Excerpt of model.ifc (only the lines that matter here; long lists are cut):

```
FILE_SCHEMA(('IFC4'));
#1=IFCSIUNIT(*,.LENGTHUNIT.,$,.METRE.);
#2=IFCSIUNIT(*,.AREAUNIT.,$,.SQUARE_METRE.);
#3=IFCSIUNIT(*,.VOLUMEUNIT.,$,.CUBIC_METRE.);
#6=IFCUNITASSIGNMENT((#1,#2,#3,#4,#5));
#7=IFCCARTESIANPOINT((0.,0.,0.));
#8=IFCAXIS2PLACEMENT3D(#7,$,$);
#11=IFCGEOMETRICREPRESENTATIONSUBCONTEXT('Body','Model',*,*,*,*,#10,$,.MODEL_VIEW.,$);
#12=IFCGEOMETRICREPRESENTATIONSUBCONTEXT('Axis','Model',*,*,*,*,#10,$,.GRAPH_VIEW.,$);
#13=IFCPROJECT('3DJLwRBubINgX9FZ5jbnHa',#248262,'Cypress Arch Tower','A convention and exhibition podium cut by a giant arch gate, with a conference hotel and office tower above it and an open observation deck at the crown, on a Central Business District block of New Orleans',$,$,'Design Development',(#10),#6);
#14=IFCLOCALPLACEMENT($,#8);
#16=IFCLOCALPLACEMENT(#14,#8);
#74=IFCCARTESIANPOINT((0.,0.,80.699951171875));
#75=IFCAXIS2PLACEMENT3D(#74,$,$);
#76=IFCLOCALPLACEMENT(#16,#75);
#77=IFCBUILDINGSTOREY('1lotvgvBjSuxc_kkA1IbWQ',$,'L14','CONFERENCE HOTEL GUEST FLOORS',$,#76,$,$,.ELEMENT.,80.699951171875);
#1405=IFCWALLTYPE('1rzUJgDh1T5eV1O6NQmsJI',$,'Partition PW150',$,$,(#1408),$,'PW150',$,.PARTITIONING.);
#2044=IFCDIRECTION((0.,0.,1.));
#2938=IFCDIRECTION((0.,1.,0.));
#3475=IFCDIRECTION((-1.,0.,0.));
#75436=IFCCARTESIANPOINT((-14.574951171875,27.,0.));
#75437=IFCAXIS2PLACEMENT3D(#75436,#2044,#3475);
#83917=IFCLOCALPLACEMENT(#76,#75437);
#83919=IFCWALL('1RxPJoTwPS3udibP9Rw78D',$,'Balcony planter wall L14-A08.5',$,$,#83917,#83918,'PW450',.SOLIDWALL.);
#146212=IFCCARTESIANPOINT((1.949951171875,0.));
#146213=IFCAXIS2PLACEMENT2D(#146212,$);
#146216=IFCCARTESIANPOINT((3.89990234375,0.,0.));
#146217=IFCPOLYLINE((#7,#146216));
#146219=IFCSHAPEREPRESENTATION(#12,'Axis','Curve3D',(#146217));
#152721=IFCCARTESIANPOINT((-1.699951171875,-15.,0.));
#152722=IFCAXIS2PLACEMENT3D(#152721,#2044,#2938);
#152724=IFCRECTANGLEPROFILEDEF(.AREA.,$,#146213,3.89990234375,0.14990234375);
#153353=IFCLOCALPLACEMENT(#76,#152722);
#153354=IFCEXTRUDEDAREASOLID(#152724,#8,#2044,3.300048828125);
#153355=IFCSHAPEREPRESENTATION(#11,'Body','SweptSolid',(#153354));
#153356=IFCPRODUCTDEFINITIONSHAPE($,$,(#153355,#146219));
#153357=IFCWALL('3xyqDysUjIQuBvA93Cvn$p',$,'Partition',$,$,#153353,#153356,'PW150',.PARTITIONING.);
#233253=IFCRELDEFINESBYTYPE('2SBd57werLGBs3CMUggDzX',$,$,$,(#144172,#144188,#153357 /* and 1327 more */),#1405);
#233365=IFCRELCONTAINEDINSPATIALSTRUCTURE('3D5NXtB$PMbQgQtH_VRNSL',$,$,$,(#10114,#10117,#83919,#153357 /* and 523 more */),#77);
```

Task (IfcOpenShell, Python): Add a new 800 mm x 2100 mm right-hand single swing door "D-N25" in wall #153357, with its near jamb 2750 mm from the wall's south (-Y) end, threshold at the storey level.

```python
import numpy as np
import ifcopenshell
import ifcopenshell.api.feature
import ifcopenshell.api.geometry
import ifcopenshell.api.root
import ifcopenshell.api.spatial
import ifcopenshell.geom
import ifcopenshell.util.element
import ifcopenshell.util.placement
import ifcopenshell.util.representation
import ifcopenshell.util.shape
import ifcopenshell.util.unit

model = ifcopenshell.open("model.ifc")
unit_scale = ifcopenshell.util.unit.calculate_unit_scale(model)
settings = ifcopenshell.geom.settings()


def volume(element):
    """Net volume in cubic metres, openings subtracted."""
    shape = ifcopenshell.geom.create_shape(settings, element)
    return ifcopenshell.util.shape.get_volume(shape.geometry)


wall = model.by_guid("3xyqDysUjIQuBvA93Cvn$p")
storey = ifcopenshell.util.element.get_container(wall, ifc_class="IfcBuildingStorey")
context = ifcopenshell.util.representation.get_context(model, "Model", "Body", "MODEL_VIEW")
before = volume(wall)

width, height, from_end, sill = 0.8, 2.1, 2.75, 0.0  # metres

# The wall runs along its own X axis, and the end named is its -X end.
wall_shape = ifcopenshell.geom.create_shape(settings, wall)
x, y, z = ifcopenshell.util.shape.get_vertices(wall_shape.geometry).T
start = x.min() + from_end
face, thickness = float(y.min()), float(y.max() - y.min())
wall_matrix = ifcopenshell.util.placement.get_local_placement(wall.ObjectPlacement)
level = ifcopenshell.util.placement.get_local_placement(storey.ObjectPlacement)[2, 3]


def in_wall(x, y):
    """Placement at x, y metres in the wall's axes, at sill height."""
    matrix = wall_matrix.copy()
    matrix[:, 3] = wall_matrix @ np.array([x / unit_scale, y / unit_scale, 0.0, 1.0])
    matrix[2, 3] = level + sill / unit_scale
    return matrix


# Opening: a box that overshoots both wall faces by 50 mm.
opening = ifcopenshell.api.root.create_entity(model, ifc_class="IfcOpeningElement", predefined_type="OPENING")
box = ifcopenshell.api.geometry.add_wall_representation(
    model, context=context, length=width, height=height, thickness=thickness + 0.1
)
ifcopenshell.api.geometry.assign_representation(model, product=opening, representation=box)
ifcopenshell.api.geometry.edit_object_placement(model, product=opening, matrix=in_wall(start, face - 0.05), is_si=False)
ifcopenshell.api.feature.add_feature(model, feature=opening, element=wall)

door = ifcopenshell.api.root.create_entity(model, ifc_class="IfcDoor", name="D-N25", predefined_type="DOOR")
door.OverallWidth, door.OverallHeight = width / unit_scale, height / unit_scale
door.OperationType = "SINGLE_SWING_RIGHT"
body = ifcopenshell.api.geometry.add_door_representation(
    model,
    context=context,
    overall_width=door.OverallWidth,
    overall_height=door.OverallHeight,
    operation_type="SINGLE_SWING_RIGHT",
    lining_properties={"LiningDepth": thickness / unit_scale, "ThresholdDepth": thickness / unit_scale},
)
ifcopenshell.api.geometry.assign_representation(model, product=door, representation=body)
ifcopenshell.api.spatial.assign_container(model, products=[door], relating_structure=storey)
ifcopenshell.api.feature.add_filling(model, opening=opening, element=door)

# The lining spans the wall, so the door starts at the wall face.
ifcopenshell.api.geometry.edit_object_placement(model, product=door, matrix=in_wall(start, face), is_si=False)

after = volume(wall)

print(f"wall volume {before:.3f} -> {after:.3f} m3")

model.write("model_edited.ifc")
```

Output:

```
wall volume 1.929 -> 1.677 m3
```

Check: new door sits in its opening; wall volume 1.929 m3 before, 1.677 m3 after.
